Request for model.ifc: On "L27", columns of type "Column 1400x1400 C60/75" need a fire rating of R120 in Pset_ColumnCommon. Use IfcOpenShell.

First a look at what the model holds.

```python
import ifcopenshell
import ifcopenshell.util.element

model = ifcopenshell.open("model.ifc")
print(model.schema)
storey = next(s for s in model.by_type("IfcBuildingStorey") if s.Name == "L27")
columns = [e for e in ifcopenshell.util.element.get_decomposition(storey) if e.is_a("IfcColumn")]
seen = {}
for e in columns:
    element_type = ifcopenshell.util.element.get_type(e)
    key = (element_type.Name if element_type != e and element_type else None, ifcopenshell.util.element.get_pset(e, "Pset_ColumnCommon", "FireRating"))
    seen[key] = seen.get(key, 0) + 1
for (name, value), count in sorted(seen.items(), key=str):
    print(count, "x", name, "|", value)
```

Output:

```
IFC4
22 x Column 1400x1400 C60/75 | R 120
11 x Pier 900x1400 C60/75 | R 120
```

```python
import ifcopenshell
import ifcopenshell.api.pset
import ifcopenshell.util.element

model = ifcopenshell.open("model.ifc")

storey = next(s for s in model.by_type("IfcBuildingStorey") if s.Name == "L27")
columns = [e for e in ifcopenshell.util.element.get_decomposition(storey) if e.is_a("IfcColumn")]

count = 0
for e in columns:
    element_type = ifcopenshell.util.element.get_type(e)
    if element_type in (None, e) or element_type.Name != "Column 1400x1400 C60/75":
        continue
    found = ifcopenshell.util.element.get_pset(e, "Pset_ColumnCommon", should_inherit=False)
    if found:
        pset = model.by_id(found["id"])
        if len(ifcopenshell.util.element.get_elements_by_pset(pset)) > 1:
            pset = ifcopenshell.api.pset.unshare_pset(model, products=[e], pset=pset)[0]
    else:
        pset = ifcopenshell.api.pset.add_pset(model, product=e, name="Pset_ColumnCommon")
    ifcopenshell.api.pset.edit_pset(model, pset=pset, properties={"FireRating": "R120"})
    count += 1

print(count, "columns updated")

model.write("model_v2.ifc")
```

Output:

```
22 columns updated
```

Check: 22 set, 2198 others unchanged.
